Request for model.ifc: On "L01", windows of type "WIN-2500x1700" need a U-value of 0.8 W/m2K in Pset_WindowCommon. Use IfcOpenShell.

First a look at what the model holds.

```python
import ifcopenshell
import ifcopenshell.util.element

model = ifcopenshell.open("model.ifc")
print(model.schema)
storey = next(s for s in model.by_type("IfcBuildingStorey") if s.Name == "L01")
windows = [e for e in ifcopenshell.util.element.get_decomposition(storey) if e.is_a("IfcWindow")]
seen = {}
for e in windows:
    element_type = ifcopenshell.util.element.get_type(e)
    key = (element_type.Name if element_type != e and element_type else None, ifcopenshell.util.element.get_pset(e, "Pset_WindowCommon", "ThermalTransmittance"))
    seen[key] = seen.get(key, 0) + 1
for (name, value), count in sorted(seen.items(), key=str):
    print(count, "x", name, "|", value)
```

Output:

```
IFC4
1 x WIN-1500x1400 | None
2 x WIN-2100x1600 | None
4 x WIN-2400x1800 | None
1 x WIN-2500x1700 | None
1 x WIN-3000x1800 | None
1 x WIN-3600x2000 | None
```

```python
import ifcopenshell
import ifcopenshell.api.pset
import ifcopenshell.util.element

model = ifcopenshell.open("model.ifc")

storey = next(s for s in model.by_type("IfcBuildingStorey") if s.Name == "L01")
windows = [e for e in ifcopenshell.util.element.get_decomposition(storey) if e.is_a("IfcWindow")]

count = 0
for e in windows:
    element_type = ifcopenshell.util.element.get_type(e)
    if element_type in (None, e) or element_type.Name != "WIN-2500x1700":
        continue
    # add_pset returns the element's existing set when there is one.
    pset = ifcopenshell.api.pset.add_pset(model, product=e, name="Pset_WindowCommon")
    ifcopenshell.api.pset.edit_pset(model, pset=pset, properties={"ThermalTransmittance": 0.8})
    count += 1

print(count, "windows updated")

model.write("model_v2.ifc")
```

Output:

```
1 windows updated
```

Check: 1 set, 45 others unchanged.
